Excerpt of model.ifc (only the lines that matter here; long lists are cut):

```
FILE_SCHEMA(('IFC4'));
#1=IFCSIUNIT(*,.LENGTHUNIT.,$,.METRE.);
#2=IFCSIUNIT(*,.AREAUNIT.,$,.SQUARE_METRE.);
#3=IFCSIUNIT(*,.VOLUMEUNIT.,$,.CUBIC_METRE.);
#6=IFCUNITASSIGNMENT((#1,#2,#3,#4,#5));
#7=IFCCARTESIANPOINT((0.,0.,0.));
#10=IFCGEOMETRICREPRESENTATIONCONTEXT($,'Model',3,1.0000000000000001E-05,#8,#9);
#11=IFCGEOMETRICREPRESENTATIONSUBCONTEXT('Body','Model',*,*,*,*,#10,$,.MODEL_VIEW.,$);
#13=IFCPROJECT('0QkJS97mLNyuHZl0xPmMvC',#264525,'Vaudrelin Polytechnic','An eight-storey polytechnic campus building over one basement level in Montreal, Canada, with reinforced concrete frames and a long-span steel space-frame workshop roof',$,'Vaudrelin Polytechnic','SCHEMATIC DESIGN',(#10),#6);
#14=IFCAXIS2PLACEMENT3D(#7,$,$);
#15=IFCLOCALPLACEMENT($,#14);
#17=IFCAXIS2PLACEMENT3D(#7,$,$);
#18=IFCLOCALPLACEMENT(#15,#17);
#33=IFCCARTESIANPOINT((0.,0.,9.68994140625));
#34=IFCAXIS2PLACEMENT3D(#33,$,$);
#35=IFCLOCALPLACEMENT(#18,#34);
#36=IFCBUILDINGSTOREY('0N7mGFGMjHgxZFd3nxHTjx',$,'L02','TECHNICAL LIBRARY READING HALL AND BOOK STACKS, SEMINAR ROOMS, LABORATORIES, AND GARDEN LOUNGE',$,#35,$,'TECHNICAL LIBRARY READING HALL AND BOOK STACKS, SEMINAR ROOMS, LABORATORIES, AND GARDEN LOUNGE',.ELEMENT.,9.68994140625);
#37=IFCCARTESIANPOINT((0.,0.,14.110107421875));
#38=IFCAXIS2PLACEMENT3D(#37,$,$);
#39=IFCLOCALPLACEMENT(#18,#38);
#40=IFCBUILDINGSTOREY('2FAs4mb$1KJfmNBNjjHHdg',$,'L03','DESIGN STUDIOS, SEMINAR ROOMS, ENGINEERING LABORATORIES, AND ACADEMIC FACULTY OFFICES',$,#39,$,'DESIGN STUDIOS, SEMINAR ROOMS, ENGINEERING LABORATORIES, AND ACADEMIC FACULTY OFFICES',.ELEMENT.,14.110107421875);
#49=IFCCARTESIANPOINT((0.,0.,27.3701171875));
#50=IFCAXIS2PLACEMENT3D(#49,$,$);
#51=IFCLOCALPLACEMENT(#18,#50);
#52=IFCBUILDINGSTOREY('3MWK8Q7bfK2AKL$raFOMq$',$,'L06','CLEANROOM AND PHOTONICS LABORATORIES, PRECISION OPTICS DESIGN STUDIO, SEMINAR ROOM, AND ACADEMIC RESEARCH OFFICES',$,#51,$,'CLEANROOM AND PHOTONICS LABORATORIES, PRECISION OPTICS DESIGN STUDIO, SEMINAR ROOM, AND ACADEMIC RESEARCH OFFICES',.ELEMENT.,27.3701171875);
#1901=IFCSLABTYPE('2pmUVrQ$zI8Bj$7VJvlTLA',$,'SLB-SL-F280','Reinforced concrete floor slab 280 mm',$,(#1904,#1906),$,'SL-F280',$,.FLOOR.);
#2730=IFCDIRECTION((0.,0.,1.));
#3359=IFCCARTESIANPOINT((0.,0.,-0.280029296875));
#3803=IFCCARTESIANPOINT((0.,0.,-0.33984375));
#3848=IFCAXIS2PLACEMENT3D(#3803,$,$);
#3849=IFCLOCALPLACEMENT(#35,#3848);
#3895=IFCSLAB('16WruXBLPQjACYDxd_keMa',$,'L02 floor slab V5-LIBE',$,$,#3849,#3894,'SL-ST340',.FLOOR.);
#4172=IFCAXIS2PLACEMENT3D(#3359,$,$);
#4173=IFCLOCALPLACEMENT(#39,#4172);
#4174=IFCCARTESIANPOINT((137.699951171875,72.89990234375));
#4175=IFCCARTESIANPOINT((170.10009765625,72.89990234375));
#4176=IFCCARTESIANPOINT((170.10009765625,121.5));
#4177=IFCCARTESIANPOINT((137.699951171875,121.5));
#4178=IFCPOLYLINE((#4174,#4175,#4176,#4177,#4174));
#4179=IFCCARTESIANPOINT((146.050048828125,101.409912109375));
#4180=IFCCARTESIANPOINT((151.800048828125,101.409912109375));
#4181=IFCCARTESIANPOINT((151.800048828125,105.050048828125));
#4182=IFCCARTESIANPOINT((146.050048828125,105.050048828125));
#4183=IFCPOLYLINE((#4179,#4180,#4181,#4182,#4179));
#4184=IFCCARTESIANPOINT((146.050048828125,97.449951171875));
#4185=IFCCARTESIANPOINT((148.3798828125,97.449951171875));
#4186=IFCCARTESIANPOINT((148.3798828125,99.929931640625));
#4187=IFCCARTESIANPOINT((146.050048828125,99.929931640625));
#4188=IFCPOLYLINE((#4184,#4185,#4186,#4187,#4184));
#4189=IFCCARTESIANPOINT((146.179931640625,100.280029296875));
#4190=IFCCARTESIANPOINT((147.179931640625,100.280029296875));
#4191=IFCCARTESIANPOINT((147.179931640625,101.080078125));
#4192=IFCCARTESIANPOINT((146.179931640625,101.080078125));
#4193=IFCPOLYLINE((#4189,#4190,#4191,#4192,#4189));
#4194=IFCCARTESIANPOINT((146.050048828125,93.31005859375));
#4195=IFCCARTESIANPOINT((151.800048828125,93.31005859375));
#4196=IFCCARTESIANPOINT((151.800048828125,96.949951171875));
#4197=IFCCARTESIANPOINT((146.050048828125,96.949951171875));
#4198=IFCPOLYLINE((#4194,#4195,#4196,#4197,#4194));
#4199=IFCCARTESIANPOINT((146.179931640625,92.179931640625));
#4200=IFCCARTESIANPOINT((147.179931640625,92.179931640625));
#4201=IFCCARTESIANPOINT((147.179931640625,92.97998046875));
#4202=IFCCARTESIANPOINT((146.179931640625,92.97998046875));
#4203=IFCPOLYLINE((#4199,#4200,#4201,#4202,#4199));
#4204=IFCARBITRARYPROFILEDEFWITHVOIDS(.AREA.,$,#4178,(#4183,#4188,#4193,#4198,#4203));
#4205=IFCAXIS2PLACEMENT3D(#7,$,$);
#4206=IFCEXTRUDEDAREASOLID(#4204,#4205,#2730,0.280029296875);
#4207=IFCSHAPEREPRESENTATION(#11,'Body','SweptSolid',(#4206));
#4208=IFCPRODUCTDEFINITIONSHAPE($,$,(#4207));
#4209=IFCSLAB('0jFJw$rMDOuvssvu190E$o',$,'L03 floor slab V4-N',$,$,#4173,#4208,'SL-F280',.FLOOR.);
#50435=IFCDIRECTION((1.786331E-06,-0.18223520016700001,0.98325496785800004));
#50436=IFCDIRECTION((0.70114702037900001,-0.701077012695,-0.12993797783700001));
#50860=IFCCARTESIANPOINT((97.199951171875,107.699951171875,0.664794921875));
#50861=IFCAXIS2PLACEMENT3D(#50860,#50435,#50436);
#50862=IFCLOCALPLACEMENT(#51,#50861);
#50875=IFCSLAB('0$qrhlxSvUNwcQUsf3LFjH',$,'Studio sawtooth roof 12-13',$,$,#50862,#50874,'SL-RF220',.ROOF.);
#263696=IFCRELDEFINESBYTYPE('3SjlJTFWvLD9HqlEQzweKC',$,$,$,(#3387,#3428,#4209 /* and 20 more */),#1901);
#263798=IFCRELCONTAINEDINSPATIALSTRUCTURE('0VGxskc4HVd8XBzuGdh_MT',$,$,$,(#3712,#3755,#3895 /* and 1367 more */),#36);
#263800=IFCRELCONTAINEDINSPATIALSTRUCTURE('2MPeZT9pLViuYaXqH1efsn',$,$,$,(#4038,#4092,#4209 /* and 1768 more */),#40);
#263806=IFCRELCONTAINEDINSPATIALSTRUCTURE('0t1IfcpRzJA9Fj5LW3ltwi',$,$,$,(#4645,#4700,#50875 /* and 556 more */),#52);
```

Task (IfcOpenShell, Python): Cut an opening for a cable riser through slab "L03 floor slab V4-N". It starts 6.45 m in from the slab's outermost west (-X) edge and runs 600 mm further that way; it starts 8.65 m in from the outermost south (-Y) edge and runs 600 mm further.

```python
import numpy as np
import ifcopenshell
import ifcopenshell.api.feature
import ifcopenshell.api.geometry
import ifcopenshell.api.root
import ifcopenshell.geom
import ifcopenshell.util.placement
import ifcopenshell.util.representation
import ifcopenshell.util.shape
import ifcopenshell.util.unit

model = ifcopenshell.open("model.ifc")
unit_scale = ifcopenshell.util.unit.calculate_unit_scale(model)
settings = ifcopenshell.geom.settings()


def volume(element):
    """Net volume in cubic metres, openings subtracted."""
    shape = ifcopenshell.geom.create_shape(settings, element)
    return ifcopenshell.util.shape.get_volume(shape.geometry)


slab = model.by_guid("0jFJw$rMDOuvssvu190E$o")
before = volume(slab)

# Extent in the slab's own axes, in metres. The edges named are its -X and -Y sides.
slab_shape = ifcopenshell.geom.create_shape(settings, slab)
vertices = ifcopenshell.util.shape.get_vertices(slab_shape.geometry)
x_min, y_min, bottom = vertices.min(axis=0)
top = vertices[:, 2].max()

opening = ifcopenshell.api.root.create_entity(model, ifc_class="IfcOpeningElement", name="Cable riser opening", predefined_type="OPENING")
context = ifcopenshell.util.representation.get_context(model, "Model", "Body", "MODEL_VIEW")
width, depth = 0.6, 0.6
outline = [(0.0, 0.0), (width, 0.0), (width, depth), (0.0, depth), (0.0, 0.0)]
# Overshoot both faces by 50 mm so the cut is clean.
shape = ifcopenshell.api.geometry.add_slab_representation(
    model, context=context, depth=top - bottom + 0.1, polyline=outline
)
ifcopenshell.api.geometry.assign_representation(model, product=opening, representation=shape)

matrix = ifcopenshell.util.placement.get_local_placement(slab.ObjectPlacement)
matrix[:, 3] = matrix @ np.append(np.array([x_min + 6.45, y_min + 8.65, bottom - 0.05]) / unit_scale, 1.0)
ifcopenshell.api.geometry.edit_object_placement(model, product=opening, matrix=matrix, is_si=False)
ifcopenshell.api.feature.add_feature(model, feature=opening, element=slab)

after = volume(slab)

print(f"slab volume {before:.3f} -> {after:.3f} m3")

model.write("model_rev.ifc")
```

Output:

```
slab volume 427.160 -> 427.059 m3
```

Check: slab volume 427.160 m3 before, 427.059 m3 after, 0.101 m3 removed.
